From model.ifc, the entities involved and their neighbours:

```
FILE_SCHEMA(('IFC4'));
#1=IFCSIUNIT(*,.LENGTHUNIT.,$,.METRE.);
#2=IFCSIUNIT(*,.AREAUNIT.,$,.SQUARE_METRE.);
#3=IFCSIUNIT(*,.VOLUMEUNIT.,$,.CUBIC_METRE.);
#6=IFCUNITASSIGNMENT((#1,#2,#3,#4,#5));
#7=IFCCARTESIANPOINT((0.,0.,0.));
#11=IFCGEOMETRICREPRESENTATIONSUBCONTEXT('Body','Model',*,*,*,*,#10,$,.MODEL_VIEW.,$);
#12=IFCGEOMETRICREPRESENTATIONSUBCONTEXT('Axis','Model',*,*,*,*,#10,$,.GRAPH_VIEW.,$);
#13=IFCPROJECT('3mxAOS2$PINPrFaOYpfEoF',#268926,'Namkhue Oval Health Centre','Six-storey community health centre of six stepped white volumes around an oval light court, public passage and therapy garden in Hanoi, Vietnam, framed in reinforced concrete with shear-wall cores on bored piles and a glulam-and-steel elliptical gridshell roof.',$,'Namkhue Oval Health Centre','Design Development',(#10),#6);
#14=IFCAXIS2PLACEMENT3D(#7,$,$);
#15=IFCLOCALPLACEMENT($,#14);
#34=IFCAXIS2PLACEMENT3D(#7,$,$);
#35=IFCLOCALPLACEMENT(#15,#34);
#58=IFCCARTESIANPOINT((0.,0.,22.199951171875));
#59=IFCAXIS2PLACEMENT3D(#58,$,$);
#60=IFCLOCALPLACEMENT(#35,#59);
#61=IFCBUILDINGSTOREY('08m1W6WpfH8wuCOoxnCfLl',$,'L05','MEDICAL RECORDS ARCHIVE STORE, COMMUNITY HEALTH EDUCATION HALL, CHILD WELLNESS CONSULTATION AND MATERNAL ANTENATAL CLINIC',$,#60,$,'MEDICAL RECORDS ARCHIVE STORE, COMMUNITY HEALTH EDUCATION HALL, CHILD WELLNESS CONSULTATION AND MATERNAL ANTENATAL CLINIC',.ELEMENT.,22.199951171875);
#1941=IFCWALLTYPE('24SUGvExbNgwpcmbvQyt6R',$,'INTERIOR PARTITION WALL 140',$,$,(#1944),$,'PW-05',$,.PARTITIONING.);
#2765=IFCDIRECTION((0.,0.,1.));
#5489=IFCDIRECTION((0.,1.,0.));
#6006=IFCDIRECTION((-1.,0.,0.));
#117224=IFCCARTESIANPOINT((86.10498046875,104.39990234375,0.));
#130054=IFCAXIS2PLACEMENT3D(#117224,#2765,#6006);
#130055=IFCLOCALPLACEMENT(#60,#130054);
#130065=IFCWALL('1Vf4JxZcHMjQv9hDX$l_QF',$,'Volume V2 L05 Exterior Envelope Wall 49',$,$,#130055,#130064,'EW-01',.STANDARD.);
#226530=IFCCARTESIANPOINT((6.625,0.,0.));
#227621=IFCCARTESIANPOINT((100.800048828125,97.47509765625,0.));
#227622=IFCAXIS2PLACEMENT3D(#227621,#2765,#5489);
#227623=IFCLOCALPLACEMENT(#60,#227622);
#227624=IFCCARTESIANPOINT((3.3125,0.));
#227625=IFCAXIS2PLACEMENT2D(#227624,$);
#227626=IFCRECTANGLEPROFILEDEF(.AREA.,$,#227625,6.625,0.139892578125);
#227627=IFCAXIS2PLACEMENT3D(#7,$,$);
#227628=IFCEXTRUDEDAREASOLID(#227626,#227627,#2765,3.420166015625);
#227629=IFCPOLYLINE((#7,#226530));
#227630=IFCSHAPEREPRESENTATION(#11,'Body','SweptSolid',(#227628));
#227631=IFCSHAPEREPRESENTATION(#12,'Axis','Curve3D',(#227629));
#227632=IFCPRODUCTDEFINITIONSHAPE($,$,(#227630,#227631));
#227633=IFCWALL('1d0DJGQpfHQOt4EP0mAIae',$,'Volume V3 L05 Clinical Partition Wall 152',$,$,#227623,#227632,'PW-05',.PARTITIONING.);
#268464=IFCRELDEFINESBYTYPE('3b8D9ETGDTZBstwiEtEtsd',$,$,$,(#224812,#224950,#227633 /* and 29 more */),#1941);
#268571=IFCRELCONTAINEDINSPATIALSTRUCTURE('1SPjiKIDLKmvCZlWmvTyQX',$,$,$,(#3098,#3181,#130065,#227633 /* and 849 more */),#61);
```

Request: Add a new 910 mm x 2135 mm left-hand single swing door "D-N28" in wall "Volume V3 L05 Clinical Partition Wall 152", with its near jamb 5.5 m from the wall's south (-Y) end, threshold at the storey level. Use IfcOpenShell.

```python
import numpy as np
import ifcopenshell
import ifcopenshell.api.feature
import ifcopenshell.api.geometry
import ifcopenshell.api.root
import ifcopenshell.api.spatial
import ifcopenshell.geom
import ifcopenshell.util.element
import ifcopenshell.util.placement
import ifcopenshell.util.representation
import ifcopenshell.util.shape
import ifcopenshell.util.unit

model = ifcopenshell.open("model.ifc")
unit_scale = ifcopenshell.util.unit.calculate_unit_scale(model)
settings = ifcopenshell.geom.settings()


def volume(element):
    """Net volume in cubic metres, openings subtracted."""
    shape = ifcopenshell.geom.create_shape(settings, element)
    return ifcopenshell.util.shape.get_volume(shape.geometry)


wall = model.by_guid("1d0DJGQpfHQOt4EP0mAIae")
storey = ifcopenshell.util.element.get_container(wall, ifc_class="IfcBuildingStorey")
context = ifcopenshell.util.representation.get_context(model, "Model", "Body", "MODEL_VIEW")
before = volume(wall)

width, height, from_end, sill = 0.91, 2.135, 5.5, 0.0  # metres

# The wall runs along its own X axis, and the end named is its -X end.
wall_shape = ifcopenshell.geom.create_shape(settings, wall)
x, y, z = ifcopenshell.util.shape.get_vertices(wall_shape.geometry).T
start = x.min() + from_end
face, thickness = float(y.min()), float(y.max() - y.min())
wall_matrix = ifcopenshell.util.placement.get_local_placement(wall.ObjectPlacement)
level = ifcopenshell.util.placement.get_local_placement(storey.ObjectPlacement)[2, 3]


def in_wall(x, y):
    """Placement at x, y metres in the wall's axes, at sill height."""
    matrix = wall_matrix.copy()
    matrix[:, 3] = wall_matrix @ np.array([x / unit_scale, y / unit_scale, 0.0, 1.0])
    matrix[2, 3] = level + sill / unit_scale
    return matrix


# Opening: a box that overshoots both wall faces by 50 mm.
opening = ifcopenshell.api.root.create_entity(model, ifc_class="IfcOpeningElement", predefined_type="OPENING")
box = ifcopenshell.api.geometry.add_wall_representation(
    model, context=context, length=width, height=height, thickness=thickness + 0.1
)
ifcopenshell.api.geometry.assign_representation(model, product=opening, representation=box)
ifcopenshell.api.geometry.edit_object_placement(model, product=opening, matrix=in_wall(start, face - 0.05), is_si=False)
ifcopenshell.api.feature.add_feature(model, feature=opening, element=wall)

door = ifcopenshell.api.root.create_entity(model, ifc_class="IfcDoor", name="D-N28", predefined_type="DOOR")
door.OverallWidth, door.OverallHeight = width / unit_scale, height / unit_scale
door.OperationType = "SINGLE_SWING_LEFT"
body = ifcopenshell.api.geometry.add_door_representation(
    model,
    context=context,
    overall_width=door.OverallWidth,
    overall_height=door.OverallHeight,
    operation_type="SINGLE_SWING_LEFT",
    lining_properties={"LiningDepth": thickness / unit_scale, "ThresholdDepth": thickness / unit_scale},
)
ifcopenshell.api.geometry.assign_representation(model, product=door, representation=body)
ifcopenshell.api.spatial.assign_container(model, products=[door], relating_structure=storey)
ifcopenshell.api.feature.add_filling(model, opening=opening, element=door)

# The lining spans the wall, so the door starts at the wall face.
ifcopenshell.api.geometry.edit_object_placement(model, product=door, matrix=in_wall(start, face), is_si=False)

after = volume(wall)

print(f"wall volume {before:.3f} -> {after:.3f} m3")

model.write("model_v2.ifc")
```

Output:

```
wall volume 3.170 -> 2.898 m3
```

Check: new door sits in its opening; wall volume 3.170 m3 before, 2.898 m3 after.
